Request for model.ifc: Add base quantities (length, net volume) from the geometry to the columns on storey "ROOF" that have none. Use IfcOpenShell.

First a look at what the model holds.

```python
import ifcopenshell
import ifcopenshell.util.element
import ifcopenshell.util.unit

model = ifcopenshell.open("model.ifc")
print(model.schema)
for unit_type in ("LENGTHUNIT", "AREAUNIT", "VOLUMEUNIT"):
    print(unit_type, ifcopenshell.util.unit.calculate_unit_scale(model, unit_type))
storey = next(s for s in model.by_type("IfcBuildingStorey") if s.Name == "ROOF")
columns = [e for e in ifcopenshell.util.element.get_decomposition(storey) if e.is_a("IfcColumn")]
for e in sorted(columns, key=lambda e: e.id()):
    print(e.id(), e.is_a(), e.Name, list(ifcopenshell.util.element.get_psets(e, qtos_only=True)), sep=" | ")
```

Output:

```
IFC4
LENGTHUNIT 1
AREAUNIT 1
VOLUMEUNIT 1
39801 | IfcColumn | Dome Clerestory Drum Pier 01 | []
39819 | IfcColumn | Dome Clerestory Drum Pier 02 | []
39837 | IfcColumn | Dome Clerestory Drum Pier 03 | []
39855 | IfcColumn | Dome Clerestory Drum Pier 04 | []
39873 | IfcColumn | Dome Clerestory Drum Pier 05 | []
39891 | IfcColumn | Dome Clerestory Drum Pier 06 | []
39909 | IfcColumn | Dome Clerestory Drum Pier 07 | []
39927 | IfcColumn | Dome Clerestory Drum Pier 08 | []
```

```python
import ifcopenshell
import ifcopenshell.api.pset
import ifcopenshell.geom
import ifcopenshell.util.element
import ifcopenshell.util.shape
import ifcopenshell.util.unit

model = ifcopenshell.open("model.ifc")
unit_scale = ifcopenshell.util.unit.calculate_unit_scale(model)
volume_scale = ifcopenshell.util.unit.calculate_unit_scale(model, "VOLUMEUNIT")
settings = ifcopenshell.geom.settings()

storey = next(s for s in model.by_type("IfcBuildingStorey") if s.Name == "ROOF")
columns = [e for e in ifcopenshell.util.element.get_decomposition(storey) if e.is_a("IfcColumn")]

for e in sorted(columns, key=lambda e: e.id()):
    if ifcopenshell.util.element.get_psets(e, qtos_only=True, should_inherit=False):
        continue
    # Geometry comes back in metres, in the element's own axes.
    shape = ifcopenshell.geom.create_shape(settings, e)
    values = {
        "Length": ifcopenshell.util.shape.get_z(shape.geometry) / unit_scale,
        "NetVolume": ifcopenshell.util.shape.get_volume(shape.geometry) / volume_scale,
    }
    qto = ifcopenshell.api.pset.add_qto(model, product=e, name="Qto_ColumnBaseQuantities")
    ifcopenshell.api.pset.edit_qto(model, qto=qto, properties=values)
    print(e.id(), {k: round(v, 3) for k, v in values.items()})

model.write("model_v2.ifc")
```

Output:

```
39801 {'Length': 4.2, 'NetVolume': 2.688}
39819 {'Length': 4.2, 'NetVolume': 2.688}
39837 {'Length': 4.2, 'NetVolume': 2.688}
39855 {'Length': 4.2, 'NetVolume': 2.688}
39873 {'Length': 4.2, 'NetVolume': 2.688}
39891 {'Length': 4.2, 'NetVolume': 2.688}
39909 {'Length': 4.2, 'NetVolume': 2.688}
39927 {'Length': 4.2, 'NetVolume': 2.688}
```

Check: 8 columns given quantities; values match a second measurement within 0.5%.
